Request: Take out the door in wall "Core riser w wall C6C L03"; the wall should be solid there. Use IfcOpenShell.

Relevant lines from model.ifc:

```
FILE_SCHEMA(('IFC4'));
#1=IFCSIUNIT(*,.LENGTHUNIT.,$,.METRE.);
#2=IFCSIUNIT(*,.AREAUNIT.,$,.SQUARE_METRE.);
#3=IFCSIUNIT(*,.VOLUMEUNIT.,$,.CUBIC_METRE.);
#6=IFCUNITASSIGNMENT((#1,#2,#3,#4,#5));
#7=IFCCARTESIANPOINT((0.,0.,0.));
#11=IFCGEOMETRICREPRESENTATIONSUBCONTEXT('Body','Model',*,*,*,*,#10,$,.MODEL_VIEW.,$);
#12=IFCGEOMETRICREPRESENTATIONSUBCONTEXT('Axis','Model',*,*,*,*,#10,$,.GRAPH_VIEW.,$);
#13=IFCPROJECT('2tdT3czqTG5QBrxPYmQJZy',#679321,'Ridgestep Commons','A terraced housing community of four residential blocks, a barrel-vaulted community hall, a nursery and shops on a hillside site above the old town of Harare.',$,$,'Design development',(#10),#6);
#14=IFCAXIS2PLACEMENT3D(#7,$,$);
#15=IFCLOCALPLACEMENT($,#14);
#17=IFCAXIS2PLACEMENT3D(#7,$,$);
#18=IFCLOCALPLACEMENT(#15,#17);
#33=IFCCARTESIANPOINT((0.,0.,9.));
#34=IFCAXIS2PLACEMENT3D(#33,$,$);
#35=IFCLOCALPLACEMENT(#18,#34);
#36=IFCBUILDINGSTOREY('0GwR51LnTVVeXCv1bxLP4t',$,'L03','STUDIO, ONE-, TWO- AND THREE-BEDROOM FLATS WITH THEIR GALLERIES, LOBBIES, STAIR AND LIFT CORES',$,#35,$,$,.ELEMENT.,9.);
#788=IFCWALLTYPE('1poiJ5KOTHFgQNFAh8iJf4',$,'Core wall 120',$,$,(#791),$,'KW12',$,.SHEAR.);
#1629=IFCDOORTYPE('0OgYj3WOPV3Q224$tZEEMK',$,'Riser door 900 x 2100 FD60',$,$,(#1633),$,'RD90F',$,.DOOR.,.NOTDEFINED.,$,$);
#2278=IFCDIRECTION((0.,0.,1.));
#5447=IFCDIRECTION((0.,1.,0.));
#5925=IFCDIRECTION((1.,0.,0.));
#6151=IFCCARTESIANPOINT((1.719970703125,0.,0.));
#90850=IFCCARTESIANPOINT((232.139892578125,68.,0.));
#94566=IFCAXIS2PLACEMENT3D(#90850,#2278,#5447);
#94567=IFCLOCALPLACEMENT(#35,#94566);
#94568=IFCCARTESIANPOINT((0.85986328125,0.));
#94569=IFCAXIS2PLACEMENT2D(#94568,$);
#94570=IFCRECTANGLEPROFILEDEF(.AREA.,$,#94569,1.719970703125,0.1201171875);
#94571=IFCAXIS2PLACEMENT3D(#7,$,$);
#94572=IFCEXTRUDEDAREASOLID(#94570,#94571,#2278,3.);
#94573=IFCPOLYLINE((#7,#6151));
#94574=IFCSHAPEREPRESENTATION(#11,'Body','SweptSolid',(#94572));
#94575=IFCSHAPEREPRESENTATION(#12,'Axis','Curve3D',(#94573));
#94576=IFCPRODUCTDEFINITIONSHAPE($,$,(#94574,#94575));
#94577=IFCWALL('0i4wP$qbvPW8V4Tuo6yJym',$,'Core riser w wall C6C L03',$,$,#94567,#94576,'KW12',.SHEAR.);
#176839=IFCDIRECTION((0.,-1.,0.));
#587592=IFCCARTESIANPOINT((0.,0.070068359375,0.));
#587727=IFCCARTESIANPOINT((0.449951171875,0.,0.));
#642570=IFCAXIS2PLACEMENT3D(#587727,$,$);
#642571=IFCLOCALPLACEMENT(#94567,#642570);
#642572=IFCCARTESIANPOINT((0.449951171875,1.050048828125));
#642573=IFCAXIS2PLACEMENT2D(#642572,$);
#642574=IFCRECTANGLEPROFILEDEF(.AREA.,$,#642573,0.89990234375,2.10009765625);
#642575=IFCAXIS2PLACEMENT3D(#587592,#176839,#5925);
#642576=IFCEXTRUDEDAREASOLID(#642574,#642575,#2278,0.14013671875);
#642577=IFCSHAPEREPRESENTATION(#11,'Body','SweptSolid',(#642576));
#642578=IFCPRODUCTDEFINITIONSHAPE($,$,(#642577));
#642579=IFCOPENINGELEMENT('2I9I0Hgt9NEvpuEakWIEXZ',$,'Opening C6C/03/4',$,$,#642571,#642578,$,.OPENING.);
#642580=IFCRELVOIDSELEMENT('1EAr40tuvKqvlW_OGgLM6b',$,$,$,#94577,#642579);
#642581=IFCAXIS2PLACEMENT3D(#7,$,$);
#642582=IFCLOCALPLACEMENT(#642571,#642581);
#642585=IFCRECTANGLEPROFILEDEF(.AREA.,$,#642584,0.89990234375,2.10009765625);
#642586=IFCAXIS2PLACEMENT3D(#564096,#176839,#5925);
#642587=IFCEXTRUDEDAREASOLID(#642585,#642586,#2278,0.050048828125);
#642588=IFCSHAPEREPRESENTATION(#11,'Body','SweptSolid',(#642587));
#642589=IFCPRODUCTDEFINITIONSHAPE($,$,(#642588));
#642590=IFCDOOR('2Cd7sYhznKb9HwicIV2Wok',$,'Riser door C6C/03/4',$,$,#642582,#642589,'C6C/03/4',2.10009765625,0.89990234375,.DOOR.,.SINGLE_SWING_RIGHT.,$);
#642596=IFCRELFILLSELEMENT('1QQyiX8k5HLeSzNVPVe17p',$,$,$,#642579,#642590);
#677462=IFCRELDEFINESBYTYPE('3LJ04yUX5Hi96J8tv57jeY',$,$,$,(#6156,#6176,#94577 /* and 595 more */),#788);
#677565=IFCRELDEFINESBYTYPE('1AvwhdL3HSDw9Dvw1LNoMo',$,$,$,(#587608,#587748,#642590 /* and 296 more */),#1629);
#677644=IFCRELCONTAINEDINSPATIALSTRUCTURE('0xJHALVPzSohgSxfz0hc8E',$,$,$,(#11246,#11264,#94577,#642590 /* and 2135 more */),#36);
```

```python
import ifcopenshell
import ifcopenshell.api.feature
import ifcopenshell.api.root
import ifcopenshell.geom
import ifcopenshell.util.shape

model = ifcopenshell.open("model.ifc")
settings = ifcopenshell.geom.settings()


def volume(element):
    """Net volume in cubic metres, openings subtracted."""
    shape = ifcopenshell.geom.create_shape(settings, element)
    return ifcopenshell.util.shape.get_volume(shape.geometry)


door = model.by_guid("2Cd7sYhznKb9HwicIV2Wok")
opening = door.FillsVoids[0].RelatingOpeningElement
wall = opening.VoidsElements[0].RelatingBuildingElement
before = volume(wall)

ifcopenshell.api.root.remove_product(model, product=door)
ifcopenshell.api.feature.remove_feature(model, feature=opening)

after = volume(wall)

print(f"wall volume {before:.3f} -> {after:.3f} m3")

model.write("model_v2.ifc")
```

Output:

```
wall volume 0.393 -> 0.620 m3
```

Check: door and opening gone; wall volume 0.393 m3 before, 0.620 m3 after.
